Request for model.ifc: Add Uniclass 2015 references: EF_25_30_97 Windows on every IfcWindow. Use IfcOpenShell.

First a look at what the model holds.

```python
import ifcopenshell

model = ifcopenshell.open("model.ifc")
print(model.schema)
print("classifications:", [c.Name for c in model.by_type("IfcClassification")])
for ifc_class in ("IfcDoor", "IfcRoof", "IfcStair", "IfcWall", "IfcWindow"):
    print(ifc_class, len(model.by_type(ifc_class)))
```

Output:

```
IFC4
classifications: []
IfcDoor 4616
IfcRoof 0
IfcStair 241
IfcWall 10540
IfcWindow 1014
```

```python
import ifcopenshell
import ifcopenshell.api.classification

model = ifcopenshell.open("model.ifc")

system = ifcopenshell.api.classification.add_classification(model, classification="Uniclass 2015")

codes = {
    "IfcWindow": ("EF_25_30_97", "Windows"),
}
for ifc_class, (code, name) in codes.items():
    products = model.by_type(ifc_class)
    ifcopenshell.api.classification.add_reference(
        model, products=products, classification=system, identification=code, name=name
    )
    print(code, len(products))

model.write("model-out.ifc")
```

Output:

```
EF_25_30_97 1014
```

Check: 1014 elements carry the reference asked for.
